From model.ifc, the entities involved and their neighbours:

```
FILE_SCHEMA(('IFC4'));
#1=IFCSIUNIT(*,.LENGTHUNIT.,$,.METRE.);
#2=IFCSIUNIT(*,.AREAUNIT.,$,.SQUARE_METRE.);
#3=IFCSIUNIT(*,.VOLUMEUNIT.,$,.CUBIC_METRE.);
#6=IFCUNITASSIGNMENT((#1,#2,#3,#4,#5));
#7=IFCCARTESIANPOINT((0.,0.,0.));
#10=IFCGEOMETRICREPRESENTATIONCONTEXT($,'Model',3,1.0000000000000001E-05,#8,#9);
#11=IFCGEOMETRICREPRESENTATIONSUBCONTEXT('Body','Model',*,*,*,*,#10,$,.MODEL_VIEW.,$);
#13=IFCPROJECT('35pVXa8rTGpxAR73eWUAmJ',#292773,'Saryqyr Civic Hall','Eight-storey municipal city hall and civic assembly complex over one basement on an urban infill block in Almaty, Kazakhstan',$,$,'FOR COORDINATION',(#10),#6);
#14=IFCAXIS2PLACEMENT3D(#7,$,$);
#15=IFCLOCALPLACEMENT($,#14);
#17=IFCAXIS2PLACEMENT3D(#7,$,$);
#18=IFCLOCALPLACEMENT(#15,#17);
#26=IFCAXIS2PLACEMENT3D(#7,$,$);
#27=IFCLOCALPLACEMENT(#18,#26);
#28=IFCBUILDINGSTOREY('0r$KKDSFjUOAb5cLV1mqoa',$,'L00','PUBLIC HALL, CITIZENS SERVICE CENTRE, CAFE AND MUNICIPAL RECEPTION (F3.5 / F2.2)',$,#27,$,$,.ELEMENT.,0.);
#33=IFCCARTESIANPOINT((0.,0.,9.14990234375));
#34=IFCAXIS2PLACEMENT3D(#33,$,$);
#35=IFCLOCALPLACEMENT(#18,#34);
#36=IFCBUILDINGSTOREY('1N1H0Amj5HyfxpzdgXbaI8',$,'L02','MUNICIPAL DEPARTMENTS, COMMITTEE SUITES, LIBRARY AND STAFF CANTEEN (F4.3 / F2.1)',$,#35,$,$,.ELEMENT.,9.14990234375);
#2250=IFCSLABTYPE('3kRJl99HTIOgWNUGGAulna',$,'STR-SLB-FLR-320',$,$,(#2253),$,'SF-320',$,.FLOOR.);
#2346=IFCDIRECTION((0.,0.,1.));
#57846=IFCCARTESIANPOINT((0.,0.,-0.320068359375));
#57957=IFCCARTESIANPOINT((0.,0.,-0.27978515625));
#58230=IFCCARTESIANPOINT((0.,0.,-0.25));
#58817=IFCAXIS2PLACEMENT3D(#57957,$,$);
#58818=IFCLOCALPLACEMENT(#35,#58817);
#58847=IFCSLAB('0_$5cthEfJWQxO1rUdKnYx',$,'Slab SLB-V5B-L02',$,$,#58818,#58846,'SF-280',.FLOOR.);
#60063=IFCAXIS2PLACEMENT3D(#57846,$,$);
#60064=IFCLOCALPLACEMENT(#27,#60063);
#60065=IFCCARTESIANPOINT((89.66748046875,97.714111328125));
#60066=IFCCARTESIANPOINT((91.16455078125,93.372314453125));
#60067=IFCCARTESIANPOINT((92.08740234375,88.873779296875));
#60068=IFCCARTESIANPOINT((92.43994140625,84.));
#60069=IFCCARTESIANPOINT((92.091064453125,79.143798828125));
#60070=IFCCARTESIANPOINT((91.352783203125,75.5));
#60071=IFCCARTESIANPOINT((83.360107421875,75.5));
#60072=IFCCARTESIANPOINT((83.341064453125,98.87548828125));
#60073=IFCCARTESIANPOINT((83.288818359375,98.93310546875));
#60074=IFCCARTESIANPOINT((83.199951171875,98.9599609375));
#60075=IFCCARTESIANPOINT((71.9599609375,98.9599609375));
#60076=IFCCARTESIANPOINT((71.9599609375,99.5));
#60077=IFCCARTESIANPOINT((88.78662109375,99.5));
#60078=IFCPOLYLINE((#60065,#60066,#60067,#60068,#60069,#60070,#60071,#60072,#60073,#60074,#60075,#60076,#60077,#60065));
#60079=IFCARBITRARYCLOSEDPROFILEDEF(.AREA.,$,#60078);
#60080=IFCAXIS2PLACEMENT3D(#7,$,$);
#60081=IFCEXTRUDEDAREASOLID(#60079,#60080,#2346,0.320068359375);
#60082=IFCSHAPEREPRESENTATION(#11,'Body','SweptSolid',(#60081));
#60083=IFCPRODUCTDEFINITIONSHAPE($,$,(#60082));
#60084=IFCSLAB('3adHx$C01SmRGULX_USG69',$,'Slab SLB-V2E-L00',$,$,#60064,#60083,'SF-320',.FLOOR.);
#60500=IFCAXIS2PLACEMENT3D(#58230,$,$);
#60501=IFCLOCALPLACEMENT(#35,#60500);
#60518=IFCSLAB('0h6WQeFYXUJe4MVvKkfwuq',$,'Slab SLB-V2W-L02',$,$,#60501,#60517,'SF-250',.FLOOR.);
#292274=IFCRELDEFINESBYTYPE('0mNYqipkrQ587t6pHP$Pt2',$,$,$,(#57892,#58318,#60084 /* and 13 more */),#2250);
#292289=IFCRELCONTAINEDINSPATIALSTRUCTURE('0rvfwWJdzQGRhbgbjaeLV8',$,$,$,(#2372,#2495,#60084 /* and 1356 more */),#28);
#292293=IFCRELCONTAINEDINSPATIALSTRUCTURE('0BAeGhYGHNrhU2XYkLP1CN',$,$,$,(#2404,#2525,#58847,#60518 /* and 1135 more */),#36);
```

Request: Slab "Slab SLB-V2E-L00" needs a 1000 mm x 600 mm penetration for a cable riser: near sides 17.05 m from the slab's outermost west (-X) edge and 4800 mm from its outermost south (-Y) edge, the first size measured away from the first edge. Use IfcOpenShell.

```python
import numpy as np
import ifcopenshell
import ifcopenshell.api.feature
import ifcopenshell.api.geometry
import ifcopenshell.api.root
import ifcopenshell.geom
import ifcopenshell.util.placement
import ifcopenshell.util.representation
import ifcopenshell.util.shape
import ifcopenshell.util.unit

model = ifcopenshell.open("model.ifc")
unit_scale = ifcopenshell.util.unit.calculate_unit_scale(model)
settings = ifcopenshell.geom.settings()


def volume(element):
    """Net volume in cubic metres, openings subtracted."""
    shape = ifcopenshell.geom.create_shape(settings, element)
    return ifcopenshell.util.shape.get_volume(shape.geometry)


slab = model.by_guid("3adHx$C01SmRGULX_USG69")
before = volume(slab)

# Extent in the slab's own axes, in metres. The edges named are its -X and -Y sides.
slab_shape = ifcopenshell.geom.create_shape(settings, slab)
vertices = ifcopenshell.util.shape.get_vertices(slab_shape.geometry)
x_min, y_min, bottom = vertices.min(axis=0)
top = vertices[:, 2].max()

opening = ifcopenshell.api.root.create_entity(model, ifc_class="IfcOpeningElement", name="Cable riser opening", predefined_type="OPENING")
context = ifcopenshell.util.representation.get_context(model, "Model", "Body", "MODEL_VIEW")
width, depth = 1, 0.6
outline = [(0.0, 0.0), (width, 0.0), (width, depth), (0.0, depth), (0.0, 0.0)]
# Overshoot both faces by 50 mm so the cut is clean.
shape = ifcopenshell.api.geometry.add_slab_representation(
    model, context=context, depth=top - bottom + 0.1, polyline=outline
)
ifcopenshell.api.geometry.assign_representation(model, product=opening, representation=shape)

matrix = ifcopenshell.util.placement.get_local_placement(slab.ObjectPlacement)
matrix[:, 3] = matrix @ np.append(np.array([x_min + 17.05, y_min + 4.8, bottom - 0.05]) / unit_scale, 1.0)
ifcopenshell.api.geometry.edit_object_placement(model, product=opening, matrix=matrix, is_si=False)
ifcopenshell.api.feature.add_feature(model, feature=opening, element=slab)

after = volume(slab)

print(f"slab volume {before:.3f} -> {after:.3f} m3")

model.write("model_v2.ifc")
```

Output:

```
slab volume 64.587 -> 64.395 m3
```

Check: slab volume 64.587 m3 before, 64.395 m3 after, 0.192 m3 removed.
